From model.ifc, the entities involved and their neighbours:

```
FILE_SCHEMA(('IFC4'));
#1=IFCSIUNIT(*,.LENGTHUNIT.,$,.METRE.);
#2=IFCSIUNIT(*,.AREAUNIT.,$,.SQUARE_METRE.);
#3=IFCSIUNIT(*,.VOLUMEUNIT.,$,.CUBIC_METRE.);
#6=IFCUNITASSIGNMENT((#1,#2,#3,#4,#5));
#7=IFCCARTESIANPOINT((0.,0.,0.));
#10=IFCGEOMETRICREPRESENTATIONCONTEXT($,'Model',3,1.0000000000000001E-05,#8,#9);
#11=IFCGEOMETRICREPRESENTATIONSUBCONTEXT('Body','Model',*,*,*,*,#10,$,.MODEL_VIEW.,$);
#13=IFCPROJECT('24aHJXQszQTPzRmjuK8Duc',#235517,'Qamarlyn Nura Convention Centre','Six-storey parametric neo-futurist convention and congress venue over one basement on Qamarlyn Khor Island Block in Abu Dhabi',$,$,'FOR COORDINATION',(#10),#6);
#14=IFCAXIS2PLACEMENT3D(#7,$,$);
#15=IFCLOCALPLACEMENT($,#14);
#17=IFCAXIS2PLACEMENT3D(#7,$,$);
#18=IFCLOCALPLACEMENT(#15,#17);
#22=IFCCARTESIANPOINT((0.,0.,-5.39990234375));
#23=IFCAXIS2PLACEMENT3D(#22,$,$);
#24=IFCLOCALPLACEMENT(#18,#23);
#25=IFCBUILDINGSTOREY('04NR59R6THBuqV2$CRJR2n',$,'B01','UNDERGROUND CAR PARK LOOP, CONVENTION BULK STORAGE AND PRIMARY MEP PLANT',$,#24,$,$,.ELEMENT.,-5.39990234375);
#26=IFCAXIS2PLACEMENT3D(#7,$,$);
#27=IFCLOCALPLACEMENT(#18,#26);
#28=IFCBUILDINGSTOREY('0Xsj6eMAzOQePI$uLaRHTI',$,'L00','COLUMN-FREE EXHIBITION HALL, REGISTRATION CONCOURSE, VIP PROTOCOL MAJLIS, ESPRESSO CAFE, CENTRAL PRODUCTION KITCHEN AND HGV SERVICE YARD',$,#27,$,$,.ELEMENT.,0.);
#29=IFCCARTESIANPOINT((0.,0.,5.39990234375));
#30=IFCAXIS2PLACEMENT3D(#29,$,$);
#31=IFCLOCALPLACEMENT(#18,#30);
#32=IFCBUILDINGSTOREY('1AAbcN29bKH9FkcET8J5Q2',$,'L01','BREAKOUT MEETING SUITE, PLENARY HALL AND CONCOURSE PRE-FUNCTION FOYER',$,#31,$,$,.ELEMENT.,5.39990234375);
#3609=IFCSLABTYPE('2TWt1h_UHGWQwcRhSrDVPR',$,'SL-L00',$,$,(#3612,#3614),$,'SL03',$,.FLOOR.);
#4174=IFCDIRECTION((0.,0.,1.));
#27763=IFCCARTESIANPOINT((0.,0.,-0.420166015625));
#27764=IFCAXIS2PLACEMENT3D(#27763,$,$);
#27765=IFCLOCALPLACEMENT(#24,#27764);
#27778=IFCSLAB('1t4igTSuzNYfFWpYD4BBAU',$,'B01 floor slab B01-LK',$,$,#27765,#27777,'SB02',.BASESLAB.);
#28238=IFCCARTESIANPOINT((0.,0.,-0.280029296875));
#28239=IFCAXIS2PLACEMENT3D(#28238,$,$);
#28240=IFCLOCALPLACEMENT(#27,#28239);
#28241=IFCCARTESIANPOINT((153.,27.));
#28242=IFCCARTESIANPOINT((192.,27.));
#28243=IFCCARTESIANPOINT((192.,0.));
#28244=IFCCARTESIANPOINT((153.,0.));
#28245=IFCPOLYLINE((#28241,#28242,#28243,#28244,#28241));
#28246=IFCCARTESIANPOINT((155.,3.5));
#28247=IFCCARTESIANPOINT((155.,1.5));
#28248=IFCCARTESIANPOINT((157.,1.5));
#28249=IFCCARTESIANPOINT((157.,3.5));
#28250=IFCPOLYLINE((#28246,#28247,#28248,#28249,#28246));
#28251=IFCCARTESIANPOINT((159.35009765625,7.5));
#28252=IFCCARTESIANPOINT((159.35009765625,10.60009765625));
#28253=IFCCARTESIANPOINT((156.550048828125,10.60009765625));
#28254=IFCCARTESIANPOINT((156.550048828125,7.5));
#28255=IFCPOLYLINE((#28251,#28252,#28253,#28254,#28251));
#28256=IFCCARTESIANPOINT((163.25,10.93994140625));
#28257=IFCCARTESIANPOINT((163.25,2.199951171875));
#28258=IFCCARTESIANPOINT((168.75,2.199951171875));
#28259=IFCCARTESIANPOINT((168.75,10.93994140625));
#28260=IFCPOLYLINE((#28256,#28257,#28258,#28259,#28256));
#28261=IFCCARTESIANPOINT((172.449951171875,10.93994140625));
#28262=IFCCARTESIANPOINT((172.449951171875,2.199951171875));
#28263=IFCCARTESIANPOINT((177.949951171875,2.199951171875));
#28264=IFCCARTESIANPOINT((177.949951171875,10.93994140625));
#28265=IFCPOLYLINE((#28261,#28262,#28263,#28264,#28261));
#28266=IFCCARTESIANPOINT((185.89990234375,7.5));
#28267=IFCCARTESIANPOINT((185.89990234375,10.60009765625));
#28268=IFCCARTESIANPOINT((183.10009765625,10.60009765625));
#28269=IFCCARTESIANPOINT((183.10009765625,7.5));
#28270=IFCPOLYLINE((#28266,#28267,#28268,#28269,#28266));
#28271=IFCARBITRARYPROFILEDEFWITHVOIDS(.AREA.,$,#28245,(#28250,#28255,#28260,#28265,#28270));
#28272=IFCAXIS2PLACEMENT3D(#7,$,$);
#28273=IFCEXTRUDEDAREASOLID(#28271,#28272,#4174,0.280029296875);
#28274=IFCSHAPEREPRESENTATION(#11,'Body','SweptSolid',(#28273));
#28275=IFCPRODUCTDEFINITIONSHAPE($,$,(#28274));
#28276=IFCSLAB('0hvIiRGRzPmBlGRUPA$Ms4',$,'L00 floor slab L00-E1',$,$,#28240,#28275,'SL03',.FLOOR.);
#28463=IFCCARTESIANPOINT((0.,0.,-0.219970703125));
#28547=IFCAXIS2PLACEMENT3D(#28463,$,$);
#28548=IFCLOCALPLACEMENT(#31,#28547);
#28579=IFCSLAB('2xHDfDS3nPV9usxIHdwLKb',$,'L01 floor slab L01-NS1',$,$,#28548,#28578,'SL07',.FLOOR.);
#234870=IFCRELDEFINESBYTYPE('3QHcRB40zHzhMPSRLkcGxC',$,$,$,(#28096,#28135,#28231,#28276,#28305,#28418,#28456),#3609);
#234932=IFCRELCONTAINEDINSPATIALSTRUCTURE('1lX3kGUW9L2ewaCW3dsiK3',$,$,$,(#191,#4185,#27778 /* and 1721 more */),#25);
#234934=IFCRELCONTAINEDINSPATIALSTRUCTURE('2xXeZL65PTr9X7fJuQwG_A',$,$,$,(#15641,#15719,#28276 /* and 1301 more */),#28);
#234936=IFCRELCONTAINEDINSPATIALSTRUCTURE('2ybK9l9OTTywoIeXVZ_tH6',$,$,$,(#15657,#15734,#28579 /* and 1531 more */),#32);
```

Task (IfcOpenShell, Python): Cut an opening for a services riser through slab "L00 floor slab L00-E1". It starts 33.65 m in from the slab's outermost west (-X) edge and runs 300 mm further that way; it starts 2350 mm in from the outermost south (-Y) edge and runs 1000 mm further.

```python
import numpy as np
import ifcopenshell
import ifcopenshell.api.feature
import ifcopenshell.api.geometry
import ifcopenshell.api.root
import ifcopenshell.geom
import ifcopenshell.util.placement
import ifcopenshell.util.representation
import ifcopenshell.util.shape
import ifcopenshell.util.unit

model = ifcopenshell.open("model.ifc")
unit_scale = ifcopenshell.util.unit.calculate_unit_scale(model)
settings = ifcopenshell.geom.settings()


def volume(element):
    """Net volume in cubic metres, openings subtracted."""
    shape = ifcopenshell.geom.create_shape(settings, element)
    return ifcopenshell.util.shape.get_volume(shape.geometry)


slab = model.by_id(28276)
before = volume(slab)

# Extent in the slab's own axes, in metres. The edges named are its -X and -Y sides.
slab_shape = ifcopenshell.geom.create_shape(settings, slab)
vertices = ifcopenshell.util.shape.get_vertices(slab_shape.geometry)
x_min, y_min, bottom = vertices.min(axis=0)
top = vertices[:, 2].max()

opening = ifcopenshell.api.root.create_entity(model, ifc_class="IfcOpeningElement", name="Services riser opening", predefined_type="OPENING")
context = ifcopenshell.util.representation.get_context(model, "Model", "Body", "MODEL_VIEW")
width, depth = 0.3, 1
outline = [(0.0, 0.0), (width, 0.0), (width, depth), (0.0, depth), (0.0, 0.0)]
# Overshoot both faces by 50 mm so the cut is clean.
shape = ifcopenshell.api.geometry.add_slab_representation(
    model, context=context, depth=top - bottom + 0.1, polyline=outline
)
ifcopenshell.api.geometry.assign_representation(model, product=opening, representation=shape)

matrix = ifcopenshell.util.placement.get_local_placement(slab.ObjectPlacement)
matrix[:, 3] = matrix @ np.append(np.array([x_min + 33.65, y_min + 2.35, bottom - 0.05]) / unit_scale, 1.0)
ifcopenshell.api.geometry.edit_object_placement(model, product=opening, matrix=matrix, is_si=False)
ifcopenshell.api.feature.add_feature(model, feature=opening, element=slab)

after = volume(slab)

print(f"slab volume {before:.3f} -> {after:.3f} m3")

model.write("model_v2.ifc")
```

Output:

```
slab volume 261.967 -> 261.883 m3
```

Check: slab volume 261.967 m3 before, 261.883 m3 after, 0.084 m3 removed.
